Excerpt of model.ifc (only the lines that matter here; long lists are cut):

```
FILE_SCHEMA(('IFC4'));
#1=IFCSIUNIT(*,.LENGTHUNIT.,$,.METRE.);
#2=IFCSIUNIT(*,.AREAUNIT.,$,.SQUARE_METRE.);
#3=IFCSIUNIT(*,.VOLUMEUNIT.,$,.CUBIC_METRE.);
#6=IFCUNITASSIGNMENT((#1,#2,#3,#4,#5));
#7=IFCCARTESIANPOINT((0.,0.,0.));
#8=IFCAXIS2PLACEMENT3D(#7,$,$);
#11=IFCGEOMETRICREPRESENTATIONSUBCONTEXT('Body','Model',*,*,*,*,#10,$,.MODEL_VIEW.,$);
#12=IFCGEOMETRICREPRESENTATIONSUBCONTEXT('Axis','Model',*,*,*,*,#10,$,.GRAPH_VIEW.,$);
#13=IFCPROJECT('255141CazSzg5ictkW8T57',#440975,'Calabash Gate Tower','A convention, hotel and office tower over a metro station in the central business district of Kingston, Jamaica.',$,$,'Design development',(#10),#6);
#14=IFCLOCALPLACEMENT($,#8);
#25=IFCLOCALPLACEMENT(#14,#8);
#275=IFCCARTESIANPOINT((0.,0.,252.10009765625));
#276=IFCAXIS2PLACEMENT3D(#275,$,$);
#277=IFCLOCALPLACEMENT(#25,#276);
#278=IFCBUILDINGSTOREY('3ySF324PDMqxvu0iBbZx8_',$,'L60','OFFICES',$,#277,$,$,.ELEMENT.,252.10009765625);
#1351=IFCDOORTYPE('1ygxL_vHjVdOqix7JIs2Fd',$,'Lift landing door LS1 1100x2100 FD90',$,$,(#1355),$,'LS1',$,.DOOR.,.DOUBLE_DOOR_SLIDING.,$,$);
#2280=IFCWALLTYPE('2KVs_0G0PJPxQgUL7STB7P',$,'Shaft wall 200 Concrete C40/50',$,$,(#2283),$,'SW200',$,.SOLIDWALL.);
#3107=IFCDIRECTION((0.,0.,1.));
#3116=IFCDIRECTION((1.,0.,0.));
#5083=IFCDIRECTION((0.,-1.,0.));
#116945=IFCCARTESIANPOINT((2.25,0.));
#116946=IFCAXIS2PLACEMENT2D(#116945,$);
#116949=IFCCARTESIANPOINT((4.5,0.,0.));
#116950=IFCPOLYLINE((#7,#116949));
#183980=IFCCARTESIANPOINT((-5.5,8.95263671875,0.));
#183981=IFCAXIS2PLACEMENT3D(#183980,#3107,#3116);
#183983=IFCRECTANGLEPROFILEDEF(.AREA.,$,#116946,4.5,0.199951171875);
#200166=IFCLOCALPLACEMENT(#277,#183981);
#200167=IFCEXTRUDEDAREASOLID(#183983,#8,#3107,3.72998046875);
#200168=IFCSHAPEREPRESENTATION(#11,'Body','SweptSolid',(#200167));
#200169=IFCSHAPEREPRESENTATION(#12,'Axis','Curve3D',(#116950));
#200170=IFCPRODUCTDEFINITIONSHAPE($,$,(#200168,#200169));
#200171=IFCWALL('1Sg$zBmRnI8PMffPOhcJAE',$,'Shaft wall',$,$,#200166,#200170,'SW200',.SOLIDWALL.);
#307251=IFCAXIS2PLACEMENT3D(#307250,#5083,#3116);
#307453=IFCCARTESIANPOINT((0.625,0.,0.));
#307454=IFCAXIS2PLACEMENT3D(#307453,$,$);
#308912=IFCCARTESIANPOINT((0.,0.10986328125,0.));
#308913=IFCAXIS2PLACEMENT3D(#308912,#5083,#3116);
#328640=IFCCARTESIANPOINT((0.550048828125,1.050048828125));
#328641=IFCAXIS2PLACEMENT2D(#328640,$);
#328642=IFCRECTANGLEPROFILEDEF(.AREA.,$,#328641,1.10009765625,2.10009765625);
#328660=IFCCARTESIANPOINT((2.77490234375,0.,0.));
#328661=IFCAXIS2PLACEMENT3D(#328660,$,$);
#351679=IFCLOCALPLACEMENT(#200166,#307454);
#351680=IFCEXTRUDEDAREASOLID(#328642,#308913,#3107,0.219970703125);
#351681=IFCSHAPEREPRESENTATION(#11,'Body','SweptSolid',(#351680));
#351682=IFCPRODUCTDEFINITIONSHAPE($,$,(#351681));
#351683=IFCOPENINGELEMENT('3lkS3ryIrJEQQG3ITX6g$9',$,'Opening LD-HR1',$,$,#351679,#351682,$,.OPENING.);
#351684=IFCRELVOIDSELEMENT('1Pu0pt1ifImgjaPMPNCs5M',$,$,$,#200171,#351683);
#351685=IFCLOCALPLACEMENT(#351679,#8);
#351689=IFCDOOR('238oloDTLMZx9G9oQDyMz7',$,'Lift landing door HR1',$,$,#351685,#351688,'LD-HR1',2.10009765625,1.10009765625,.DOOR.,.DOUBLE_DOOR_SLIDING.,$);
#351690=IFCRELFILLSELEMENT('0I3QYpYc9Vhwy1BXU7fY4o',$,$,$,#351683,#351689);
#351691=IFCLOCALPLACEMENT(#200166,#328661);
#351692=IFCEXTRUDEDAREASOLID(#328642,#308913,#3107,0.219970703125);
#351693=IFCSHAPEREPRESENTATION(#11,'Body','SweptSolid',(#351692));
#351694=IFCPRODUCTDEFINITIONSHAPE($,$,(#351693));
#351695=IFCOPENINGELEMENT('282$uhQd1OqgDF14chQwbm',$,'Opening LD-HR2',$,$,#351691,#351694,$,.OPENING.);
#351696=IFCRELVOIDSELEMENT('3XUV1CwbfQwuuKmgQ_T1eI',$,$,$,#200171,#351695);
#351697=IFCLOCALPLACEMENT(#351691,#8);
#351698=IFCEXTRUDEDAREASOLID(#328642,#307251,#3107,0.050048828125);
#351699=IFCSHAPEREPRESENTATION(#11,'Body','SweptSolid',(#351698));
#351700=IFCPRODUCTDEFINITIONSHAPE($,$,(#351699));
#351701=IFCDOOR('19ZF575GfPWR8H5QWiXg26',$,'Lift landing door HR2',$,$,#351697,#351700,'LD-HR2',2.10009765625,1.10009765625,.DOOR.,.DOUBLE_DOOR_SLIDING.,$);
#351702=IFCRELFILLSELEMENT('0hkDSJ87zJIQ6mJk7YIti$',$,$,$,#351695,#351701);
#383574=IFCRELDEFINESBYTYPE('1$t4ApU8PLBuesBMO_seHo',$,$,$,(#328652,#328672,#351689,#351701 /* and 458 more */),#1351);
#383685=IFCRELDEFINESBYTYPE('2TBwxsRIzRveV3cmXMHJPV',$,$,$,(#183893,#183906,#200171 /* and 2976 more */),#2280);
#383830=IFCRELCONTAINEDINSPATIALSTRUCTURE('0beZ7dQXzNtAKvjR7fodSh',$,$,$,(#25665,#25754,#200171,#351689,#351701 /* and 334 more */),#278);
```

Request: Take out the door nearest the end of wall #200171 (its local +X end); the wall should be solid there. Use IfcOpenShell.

```python
import ifcopenshell
import ifcopenshell.api.feature
import ifcopenshell.api.root
import ifcopenshell.geom
import ifcopenshell.util.shape

model = ifcopenshell.open("model.ifc")
settings = ifcopenshell.geom.settings()


def volume(element):
    """Net volume in cubic metres, openings subtracted."""
    shape = ifcopenshell.geom.create_shape(settings, element)
    return ifcopenshell.util.shape.get_volume(shape.geometry)


door = model.by_id(351701)
opening = door.FillsVoids[0].RelatingOpeningElement
wall = opening.VoidsElements[0].RelatingBuildingElement
before = volume(wall)

ifcopenshell.api.root.remove_product(model, product=door)
ifcopenshell.api.feature.remove_feature(model, feature=opening)

after = volume(wall)

print(f"wall volume {before:.3f} -> {after:.3f} m3")

model.write("model_updated.ifc")
```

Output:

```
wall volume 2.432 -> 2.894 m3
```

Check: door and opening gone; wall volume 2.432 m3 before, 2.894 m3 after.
